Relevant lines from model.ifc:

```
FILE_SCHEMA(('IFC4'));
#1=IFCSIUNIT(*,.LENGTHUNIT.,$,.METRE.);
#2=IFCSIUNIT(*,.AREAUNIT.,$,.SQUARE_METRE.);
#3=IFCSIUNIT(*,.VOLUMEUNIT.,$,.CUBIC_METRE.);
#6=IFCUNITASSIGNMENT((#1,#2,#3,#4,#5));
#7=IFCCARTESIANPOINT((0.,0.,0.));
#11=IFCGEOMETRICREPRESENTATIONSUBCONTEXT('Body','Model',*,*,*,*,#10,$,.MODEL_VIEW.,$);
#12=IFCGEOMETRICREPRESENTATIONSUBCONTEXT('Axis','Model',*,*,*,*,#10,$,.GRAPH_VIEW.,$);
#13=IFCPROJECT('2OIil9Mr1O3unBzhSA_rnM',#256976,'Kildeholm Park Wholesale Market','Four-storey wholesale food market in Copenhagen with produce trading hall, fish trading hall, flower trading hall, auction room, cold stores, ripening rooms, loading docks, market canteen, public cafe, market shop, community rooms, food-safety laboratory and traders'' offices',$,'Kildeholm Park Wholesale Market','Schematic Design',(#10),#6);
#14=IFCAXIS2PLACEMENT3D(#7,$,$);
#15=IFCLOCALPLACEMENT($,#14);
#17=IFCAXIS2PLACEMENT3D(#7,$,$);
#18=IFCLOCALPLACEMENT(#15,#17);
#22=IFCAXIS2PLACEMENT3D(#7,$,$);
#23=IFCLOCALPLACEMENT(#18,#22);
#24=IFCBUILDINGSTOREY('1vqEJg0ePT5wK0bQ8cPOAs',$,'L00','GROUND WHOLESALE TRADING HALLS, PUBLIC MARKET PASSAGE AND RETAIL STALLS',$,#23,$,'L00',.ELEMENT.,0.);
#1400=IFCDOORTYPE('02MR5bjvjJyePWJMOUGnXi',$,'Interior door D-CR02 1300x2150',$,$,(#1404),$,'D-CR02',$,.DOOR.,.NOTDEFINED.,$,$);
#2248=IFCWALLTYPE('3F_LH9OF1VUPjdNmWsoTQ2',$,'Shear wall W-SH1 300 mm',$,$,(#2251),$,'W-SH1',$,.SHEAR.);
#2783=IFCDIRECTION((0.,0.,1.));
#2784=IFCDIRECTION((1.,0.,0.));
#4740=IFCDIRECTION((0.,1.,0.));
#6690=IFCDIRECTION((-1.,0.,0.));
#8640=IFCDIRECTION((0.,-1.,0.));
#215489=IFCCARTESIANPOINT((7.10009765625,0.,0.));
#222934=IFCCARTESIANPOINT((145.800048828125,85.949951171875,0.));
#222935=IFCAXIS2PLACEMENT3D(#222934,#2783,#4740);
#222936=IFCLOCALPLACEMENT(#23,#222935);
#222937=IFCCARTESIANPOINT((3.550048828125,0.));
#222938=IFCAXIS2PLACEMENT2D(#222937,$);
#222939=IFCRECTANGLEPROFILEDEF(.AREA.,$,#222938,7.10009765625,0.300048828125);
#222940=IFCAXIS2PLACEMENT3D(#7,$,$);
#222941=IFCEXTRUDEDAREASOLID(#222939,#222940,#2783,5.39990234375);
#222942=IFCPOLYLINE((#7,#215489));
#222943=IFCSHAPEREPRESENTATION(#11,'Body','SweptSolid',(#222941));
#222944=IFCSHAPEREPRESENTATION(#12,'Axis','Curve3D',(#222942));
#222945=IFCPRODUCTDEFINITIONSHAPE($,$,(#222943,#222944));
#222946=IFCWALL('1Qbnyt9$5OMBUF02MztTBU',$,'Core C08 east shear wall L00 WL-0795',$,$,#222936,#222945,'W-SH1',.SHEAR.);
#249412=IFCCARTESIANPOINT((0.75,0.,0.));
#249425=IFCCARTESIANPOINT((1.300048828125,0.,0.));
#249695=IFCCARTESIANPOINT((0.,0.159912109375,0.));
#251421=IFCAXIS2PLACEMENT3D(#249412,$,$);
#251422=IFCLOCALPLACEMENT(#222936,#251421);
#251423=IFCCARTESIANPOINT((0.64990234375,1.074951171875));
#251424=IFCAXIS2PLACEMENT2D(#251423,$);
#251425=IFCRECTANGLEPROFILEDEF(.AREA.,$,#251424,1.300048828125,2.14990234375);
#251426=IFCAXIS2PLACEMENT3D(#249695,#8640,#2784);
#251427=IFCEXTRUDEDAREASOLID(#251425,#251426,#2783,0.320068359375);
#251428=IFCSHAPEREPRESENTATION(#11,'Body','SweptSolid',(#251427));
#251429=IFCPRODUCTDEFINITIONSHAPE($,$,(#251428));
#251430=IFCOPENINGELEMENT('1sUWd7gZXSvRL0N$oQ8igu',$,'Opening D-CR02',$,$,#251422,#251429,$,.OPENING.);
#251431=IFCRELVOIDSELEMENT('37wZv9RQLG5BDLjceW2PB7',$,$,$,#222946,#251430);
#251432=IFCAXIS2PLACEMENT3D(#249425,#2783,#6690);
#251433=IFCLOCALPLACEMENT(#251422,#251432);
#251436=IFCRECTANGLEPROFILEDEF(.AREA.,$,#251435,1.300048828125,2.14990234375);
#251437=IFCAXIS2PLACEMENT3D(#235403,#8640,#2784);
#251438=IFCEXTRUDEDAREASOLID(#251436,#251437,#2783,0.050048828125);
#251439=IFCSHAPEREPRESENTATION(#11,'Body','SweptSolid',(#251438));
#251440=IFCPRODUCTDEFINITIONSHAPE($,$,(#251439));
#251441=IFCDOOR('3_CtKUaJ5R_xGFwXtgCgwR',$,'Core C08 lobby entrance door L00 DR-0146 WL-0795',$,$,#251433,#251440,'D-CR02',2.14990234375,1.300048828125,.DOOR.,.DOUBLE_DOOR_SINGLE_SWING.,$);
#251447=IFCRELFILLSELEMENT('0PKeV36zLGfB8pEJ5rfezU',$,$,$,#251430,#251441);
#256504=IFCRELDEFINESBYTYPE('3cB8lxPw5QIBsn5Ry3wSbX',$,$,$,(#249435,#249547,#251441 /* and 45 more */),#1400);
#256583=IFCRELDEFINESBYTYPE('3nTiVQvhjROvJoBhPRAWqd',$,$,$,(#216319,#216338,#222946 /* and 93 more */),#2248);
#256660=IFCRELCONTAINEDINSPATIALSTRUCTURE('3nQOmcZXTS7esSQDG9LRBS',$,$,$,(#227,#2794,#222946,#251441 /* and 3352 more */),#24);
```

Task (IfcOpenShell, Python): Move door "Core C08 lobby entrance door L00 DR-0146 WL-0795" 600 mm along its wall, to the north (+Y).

```python
import ifcopenshell
import ifcopenshell.api.geometry
import ifcopenshell.util.placement
import ifcopenshell.util.unit

model = ifcopenshell.open("model.ifc")
unit_scale = ifcopenshell.util.unit.calculate_unit_scale(model)

door = model.by_id(251441)
opening = door.FillsVoids[0].RelatingOpeningElement
wall = opening.VoidsElements[0].RelatingBuildingElement

wall_matrix = ifcopenshell.util.placement.get_local_placement(wall.ObjectPlacement)
shift = wall_matrix[:3, 0] * 0.6 / unit_scale
before = ifcopenshell.util.placement.get_local_placement(door.ObjectPlacement)[:3, 3].copy()

# The door is placed relative to its opening, so it follows when the opening moves.
matrix = ifcopenshell.util.placement.get_local_placement(opening.ObjectPlacement)
matrix[:3, 3] += shift
ifcopenshell.api.geometry.edit_object_placement(
    model, product=opening, matrix=matrix, is_si=False, should_transform_children=True
)

after = ifcopenshell.util.placement.get_local_placement(door.ObjectPlacement)[:3, 3]
print("door moved by", (after - before).round(3) + 0.0)

model.write("model_edited.ifc")
```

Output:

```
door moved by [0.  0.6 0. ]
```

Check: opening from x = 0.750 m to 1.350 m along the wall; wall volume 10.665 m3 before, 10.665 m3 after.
